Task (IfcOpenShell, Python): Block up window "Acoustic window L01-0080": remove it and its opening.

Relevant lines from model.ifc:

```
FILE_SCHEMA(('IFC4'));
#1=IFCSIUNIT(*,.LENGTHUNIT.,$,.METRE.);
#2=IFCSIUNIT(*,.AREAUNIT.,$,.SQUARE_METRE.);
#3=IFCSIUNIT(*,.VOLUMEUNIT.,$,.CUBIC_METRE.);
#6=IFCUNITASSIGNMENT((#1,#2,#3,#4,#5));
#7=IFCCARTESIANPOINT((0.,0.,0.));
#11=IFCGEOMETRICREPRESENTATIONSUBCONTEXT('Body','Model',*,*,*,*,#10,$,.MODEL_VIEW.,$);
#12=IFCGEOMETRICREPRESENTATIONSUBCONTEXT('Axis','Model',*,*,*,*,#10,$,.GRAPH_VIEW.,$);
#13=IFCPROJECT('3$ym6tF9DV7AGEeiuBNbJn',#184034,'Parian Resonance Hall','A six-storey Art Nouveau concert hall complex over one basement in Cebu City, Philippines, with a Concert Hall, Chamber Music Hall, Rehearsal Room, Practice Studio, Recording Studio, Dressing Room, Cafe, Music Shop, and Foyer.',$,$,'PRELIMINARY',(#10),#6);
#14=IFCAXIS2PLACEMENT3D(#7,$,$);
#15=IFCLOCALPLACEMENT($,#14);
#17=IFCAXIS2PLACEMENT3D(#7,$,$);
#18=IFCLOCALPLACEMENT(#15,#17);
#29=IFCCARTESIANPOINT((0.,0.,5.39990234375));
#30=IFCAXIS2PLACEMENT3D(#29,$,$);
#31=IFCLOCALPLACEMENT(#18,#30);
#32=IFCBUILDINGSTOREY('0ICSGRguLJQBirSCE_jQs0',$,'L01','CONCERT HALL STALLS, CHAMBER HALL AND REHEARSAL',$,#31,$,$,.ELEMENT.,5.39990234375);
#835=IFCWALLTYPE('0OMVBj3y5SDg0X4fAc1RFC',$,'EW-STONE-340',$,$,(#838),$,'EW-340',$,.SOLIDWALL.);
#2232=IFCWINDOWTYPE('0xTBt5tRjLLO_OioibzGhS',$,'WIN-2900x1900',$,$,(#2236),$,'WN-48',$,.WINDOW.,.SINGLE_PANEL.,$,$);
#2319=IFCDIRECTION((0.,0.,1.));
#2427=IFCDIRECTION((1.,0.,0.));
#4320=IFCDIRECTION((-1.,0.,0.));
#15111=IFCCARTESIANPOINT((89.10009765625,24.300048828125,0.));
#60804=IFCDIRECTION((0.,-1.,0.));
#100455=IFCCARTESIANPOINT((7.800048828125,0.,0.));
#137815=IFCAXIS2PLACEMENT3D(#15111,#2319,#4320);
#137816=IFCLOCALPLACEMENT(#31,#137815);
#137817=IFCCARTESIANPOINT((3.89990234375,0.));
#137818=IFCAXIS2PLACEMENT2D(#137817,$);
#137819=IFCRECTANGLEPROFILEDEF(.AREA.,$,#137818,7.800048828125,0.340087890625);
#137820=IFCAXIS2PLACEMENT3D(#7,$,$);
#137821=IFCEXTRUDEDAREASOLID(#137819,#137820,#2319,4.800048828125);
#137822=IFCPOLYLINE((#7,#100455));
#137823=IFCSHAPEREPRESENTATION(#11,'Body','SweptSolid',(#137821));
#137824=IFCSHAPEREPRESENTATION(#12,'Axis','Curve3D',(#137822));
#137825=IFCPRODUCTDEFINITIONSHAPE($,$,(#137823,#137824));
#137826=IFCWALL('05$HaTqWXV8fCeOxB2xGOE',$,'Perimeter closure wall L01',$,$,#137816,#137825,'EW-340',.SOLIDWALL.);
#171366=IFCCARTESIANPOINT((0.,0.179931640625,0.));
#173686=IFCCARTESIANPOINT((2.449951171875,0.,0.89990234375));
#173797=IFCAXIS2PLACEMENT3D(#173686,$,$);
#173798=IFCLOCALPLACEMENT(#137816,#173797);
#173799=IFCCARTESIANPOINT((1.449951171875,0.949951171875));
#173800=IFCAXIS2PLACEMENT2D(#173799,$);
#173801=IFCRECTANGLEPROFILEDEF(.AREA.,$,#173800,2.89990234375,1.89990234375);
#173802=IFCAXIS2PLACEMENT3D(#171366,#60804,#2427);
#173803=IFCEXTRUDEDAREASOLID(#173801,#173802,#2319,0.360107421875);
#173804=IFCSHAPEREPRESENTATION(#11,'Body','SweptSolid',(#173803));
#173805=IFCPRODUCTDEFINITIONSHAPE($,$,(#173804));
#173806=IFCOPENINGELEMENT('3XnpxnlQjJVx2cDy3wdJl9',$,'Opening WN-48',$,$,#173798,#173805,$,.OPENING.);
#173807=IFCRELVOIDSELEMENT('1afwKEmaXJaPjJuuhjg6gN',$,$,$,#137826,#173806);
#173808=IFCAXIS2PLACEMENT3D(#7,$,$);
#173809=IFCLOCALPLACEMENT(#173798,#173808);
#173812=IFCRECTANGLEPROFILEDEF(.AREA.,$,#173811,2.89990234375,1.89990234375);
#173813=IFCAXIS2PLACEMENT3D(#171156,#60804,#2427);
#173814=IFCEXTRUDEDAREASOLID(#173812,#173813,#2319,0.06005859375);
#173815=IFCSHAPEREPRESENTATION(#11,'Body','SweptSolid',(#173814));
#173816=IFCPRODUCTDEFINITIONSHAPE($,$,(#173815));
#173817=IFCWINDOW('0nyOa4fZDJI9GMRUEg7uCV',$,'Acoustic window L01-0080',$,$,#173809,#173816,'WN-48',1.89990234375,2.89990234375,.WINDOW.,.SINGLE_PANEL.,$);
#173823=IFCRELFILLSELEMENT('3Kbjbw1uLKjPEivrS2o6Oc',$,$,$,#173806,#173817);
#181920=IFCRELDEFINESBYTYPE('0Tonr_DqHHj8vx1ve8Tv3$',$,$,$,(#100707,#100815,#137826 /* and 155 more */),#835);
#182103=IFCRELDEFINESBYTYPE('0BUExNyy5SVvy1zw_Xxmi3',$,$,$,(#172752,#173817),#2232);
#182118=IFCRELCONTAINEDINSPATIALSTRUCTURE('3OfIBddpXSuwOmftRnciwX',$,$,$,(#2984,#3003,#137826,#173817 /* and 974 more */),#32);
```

```python
import ifcopenshell
import ifcopenshell.api.feature
import ifcopenshell.api.root
import ifcopenshell.geom
import ifcopenshell.util.shape

model = ifcopenshell.open("model.ifc")
settings = ifcopenshell.geom.settings()


def volume(element):
    """Net volume in cubic metres, openings subtracted."""
    shape = ifcopenshell.geom.create_shape(settings, element)
    return ifcopenshell.util.shape.get_volume(shape.geometry)


window = model.by_guid("0nyOa4fZDJI9GMRUEg7uCV")
opening = window.FillsVoids[0].RelatingOpeningElement
wall = opening.VoidsElements[0].RelatingBuildingElement
before = volume(wall)

ifcopenshell.api.root.remove_product(model, product=window)
ifcopenshell.api.feature.remove_feature(model, feature=opening)

after = volume(wall)

print(f"wall volume {before:.3f} -> {after:.3f} m3")

model.write("model_v2.ifc")
```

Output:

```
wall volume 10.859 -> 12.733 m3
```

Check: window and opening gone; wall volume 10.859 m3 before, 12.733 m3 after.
